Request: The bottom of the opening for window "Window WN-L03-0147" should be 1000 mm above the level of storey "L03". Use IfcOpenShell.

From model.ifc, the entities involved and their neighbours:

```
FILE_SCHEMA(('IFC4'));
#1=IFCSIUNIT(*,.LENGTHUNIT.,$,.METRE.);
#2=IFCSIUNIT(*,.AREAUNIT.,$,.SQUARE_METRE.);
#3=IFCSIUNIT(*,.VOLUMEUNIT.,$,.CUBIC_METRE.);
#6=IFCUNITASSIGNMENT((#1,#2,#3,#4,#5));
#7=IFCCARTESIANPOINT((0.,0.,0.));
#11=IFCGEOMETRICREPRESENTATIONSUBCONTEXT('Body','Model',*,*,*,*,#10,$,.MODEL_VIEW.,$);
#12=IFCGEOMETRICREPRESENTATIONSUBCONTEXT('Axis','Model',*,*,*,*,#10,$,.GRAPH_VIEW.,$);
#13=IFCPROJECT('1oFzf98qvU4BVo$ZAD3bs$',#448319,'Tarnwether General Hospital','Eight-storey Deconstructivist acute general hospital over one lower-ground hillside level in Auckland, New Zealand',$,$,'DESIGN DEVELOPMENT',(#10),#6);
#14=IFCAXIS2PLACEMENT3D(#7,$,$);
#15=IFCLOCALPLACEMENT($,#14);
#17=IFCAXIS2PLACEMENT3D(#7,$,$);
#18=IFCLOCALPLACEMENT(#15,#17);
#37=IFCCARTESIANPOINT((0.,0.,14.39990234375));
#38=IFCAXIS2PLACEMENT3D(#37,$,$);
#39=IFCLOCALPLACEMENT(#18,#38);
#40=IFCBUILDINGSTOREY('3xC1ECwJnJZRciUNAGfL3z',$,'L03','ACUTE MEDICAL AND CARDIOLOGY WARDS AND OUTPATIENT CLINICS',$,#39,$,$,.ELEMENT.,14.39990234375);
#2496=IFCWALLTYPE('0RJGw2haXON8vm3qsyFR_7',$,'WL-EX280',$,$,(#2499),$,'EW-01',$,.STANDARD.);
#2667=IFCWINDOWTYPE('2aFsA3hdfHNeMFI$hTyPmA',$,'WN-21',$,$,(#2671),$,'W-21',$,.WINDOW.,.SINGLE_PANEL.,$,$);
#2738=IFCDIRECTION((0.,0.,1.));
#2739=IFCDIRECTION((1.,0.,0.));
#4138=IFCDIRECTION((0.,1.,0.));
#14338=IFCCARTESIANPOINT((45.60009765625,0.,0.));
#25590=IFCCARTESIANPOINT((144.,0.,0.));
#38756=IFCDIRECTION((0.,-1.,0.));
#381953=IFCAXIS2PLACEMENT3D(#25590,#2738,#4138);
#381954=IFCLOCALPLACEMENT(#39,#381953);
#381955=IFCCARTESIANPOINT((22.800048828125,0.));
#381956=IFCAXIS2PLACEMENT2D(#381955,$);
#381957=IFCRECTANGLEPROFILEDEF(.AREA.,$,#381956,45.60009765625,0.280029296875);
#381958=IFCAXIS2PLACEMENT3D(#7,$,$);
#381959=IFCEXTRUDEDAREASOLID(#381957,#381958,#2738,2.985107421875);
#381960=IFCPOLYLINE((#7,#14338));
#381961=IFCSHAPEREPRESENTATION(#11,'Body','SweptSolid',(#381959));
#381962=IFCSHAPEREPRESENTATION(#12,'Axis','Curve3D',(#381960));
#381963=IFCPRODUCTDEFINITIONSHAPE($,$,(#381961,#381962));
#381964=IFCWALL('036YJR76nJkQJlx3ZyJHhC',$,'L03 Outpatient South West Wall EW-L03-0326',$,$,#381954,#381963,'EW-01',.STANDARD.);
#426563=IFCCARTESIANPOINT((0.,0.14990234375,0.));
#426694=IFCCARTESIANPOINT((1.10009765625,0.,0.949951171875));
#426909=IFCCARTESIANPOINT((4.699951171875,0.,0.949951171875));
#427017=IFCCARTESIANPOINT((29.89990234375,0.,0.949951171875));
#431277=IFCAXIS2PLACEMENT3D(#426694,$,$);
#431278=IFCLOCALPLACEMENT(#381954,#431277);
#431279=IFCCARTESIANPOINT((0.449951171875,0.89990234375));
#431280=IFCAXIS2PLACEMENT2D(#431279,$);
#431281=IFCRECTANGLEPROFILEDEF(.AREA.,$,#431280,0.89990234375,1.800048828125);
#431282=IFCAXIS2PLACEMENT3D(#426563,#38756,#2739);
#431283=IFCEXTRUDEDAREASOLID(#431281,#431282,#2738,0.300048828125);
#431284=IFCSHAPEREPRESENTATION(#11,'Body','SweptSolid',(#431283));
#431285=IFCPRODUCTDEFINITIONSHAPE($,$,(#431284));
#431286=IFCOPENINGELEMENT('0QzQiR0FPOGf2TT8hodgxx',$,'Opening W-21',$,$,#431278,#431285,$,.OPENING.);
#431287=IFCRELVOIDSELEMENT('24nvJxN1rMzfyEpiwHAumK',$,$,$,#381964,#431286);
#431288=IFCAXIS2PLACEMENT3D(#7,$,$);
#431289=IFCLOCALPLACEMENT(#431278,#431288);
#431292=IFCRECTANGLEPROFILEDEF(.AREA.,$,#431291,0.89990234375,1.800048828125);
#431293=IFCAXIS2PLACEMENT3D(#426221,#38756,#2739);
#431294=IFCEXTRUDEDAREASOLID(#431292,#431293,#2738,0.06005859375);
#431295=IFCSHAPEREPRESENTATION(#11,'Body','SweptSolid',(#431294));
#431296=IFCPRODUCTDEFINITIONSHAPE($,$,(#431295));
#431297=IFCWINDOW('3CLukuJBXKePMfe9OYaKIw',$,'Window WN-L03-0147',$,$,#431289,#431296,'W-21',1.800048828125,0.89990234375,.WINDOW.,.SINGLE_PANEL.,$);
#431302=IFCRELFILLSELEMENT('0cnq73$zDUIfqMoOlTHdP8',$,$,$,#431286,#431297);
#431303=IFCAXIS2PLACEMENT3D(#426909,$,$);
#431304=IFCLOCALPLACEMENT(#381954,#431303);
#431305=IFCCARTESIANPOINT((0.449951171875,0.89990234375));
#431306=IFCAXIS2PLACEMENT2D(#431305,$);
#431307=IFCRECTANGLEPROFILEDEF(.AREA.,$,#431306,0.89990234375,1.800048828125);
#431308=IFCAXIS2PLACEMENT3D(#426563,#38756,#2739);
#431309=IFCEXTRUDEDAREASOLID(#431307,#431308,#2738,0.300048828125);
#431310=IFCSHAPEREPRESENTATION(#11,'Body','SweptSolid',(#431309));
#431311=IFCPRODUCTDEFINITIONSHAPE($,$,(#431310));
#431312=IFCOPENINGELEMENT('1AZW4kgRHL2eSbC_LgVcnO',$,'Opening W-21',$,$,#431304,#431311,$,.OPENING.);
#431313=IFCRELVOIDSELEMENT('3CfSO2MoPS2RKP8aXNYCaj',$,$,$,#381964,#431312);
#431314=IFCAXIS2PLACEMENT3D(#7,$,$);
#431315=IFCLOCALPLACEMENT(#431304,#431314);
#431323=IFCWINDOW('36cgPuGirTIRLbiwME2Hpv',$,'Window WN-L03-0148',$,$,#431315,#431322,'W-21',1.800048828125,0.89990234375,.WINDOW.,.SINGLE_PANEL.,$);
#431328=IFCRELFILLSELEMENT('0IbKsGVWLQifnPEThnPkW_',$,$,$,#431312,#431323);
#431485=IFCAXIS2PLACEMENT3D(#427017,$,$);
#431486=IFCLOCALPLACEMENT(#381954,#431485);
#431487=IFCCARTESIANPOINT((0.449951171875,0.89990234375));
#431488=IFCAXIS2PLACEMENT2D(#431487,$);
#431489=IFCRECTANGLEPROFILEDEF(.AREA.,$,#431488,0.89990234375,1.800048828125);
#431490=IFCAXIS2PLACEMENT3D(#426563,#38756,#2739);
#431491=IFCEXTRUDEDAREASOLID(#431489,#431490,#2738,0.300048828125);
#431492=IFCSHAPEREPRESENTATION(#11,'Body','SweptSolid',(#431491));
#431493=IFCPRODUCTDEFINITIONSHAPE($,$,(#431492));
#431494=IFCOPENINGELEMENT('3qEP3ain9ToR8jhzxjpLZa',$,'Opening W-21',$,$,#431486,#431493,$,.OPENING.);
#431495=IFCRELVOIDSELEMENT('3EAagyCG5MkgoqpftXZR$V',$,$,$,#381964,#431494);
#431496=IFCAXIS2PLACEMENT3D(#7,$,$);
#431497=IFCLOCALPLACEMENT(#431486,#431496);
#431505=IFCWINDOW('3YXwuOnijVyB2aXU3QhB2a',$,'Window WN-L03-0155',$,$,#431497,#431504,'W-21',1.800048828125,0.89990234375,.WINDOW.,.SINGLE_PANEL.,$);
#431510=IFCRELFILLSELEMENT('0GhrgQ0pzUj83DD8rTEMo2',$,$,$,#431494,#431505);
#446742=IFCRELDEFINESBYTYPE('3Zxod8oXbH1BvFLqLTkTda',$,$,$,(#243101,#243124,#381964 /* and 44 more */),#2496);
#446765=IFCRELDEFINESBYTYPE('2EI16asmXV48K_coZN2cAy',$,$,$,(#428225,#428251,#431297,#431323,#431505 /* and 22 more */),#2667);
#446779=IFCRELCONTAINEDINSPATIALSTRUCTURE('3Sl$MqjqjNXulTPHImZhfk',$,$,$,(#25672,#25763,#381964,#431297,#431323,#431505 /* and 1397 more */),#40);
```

```python
import numpy as np
import ifcopenshell
import ifcopenshell.api.geometry
import ifcopenshell.geom
import ifcopenshell.util.element
import ifcopenshell.util.placement
import ifcopenshell.util.shape
import ifcopenshell.util.unit

model = ifcopenshell.open("model.ifc")
unit_scale = ifcopenshell.util.unit.calculate_unit_scale(model)

window = model.by_id(431297)
opening = window.FillsVoids[0].RelatingOpeningElement
storey = ifcopenshell.util.element.get_container(window, ifc_class="IfcBuildingStorey")
level = ifcopenshell.util.placement.get_local_placement(storey.ObjectPlacement)[2, 3]

# The opening's origin need not be at the sill, so measure its lowest point.
shape = ifcopenshell.geom.create_shape(ifcopenshell.geom.settings(), opening)
bottom = ifcopenshell.util.shape.get_shape_bottom_elevation(shape, shape.geometry) / unit_scale
dz = level + 1 / unit_scale - bottom

shift = np.array([0.0, 0.0, dz])
# The window is placed relative to its opening, so it follows when the opening moves.
matrix = ifcopenshell.util.placement.get_local_placement(opening.ObjectPlacement)
matrix[:3, 3] += shift
ifcopenshell.api.geometry.edit_object_placement(
    model, product=opening, matrix=matrix, is_si=False, should_transform_children=True
)

print(f"moved by {dz * unit_scale:+.3f} m")

model.write("model_edited.ifc")
```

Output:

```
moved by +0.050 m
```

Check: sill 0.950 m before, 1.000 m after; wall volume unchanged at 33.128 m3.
